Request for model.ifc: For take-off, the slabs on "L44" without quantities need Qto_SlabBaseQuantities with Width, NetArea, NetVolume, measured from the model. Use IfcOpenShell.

First a look at what the model holds.

```python
import ifcopenshell
import ifcopenshell.util.element
import ifcopenshell.util.unit

model = ifcopenshell.open("model.ifc")
print(model.schema)
for unit_type in ("LENGTHUNIT", "AREAUNIT", "VOLUMEUNIT"):
    print(unit_type, ifcopenshell.util.unit.calculate_unit_scale(model, unit_type))
storey = next(s for s in model.by_type("IfcBuildingStorey") if s.Name == "L44")
slabs = [e for e in ifcopenshell.util.element.get_decomposition(storey) if e.is_a("IfcSlab")]
for e in sorted(slabs, key=lambda e: e.id()):
    print(e.id(), e.is_a(), e.Name, list(ifcopenshell.util.element.get_psets(e, qtos_only=True)), sep=" | ")
```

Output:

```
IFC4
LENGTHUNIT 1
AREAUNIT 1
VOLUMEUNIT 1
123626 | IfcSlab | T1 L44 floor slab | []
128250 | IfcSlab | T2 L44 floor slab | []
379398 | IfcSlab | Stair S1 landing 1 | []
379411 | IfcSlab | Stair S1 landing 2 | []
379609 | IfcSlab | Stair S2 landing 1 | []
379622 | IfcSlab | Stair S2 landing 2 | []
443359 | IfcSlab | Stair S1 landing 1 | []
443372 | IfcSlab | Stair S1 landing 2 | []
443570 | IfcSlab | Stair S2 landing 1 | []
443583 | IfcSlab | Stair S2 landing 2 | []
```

```python
import ifcopenshell
import ifcopenshell.api.pset
import ifcopenshell.geom
import ifcopenshell.util.element
import ifcopenshell.util.shape
import ifcopenshell.util.unit

model = ifcopenshell.open("model.ifc")
unit_scale = ifcopenshell.util.unit.calculate_unit_scale(model)
area_scale = ifcopenshell.util.unit.calculate_unit_scale(model, "AREAUNIT")
volume_scale = ifcopenshell.util.unit.calculate_unit_scale(model, "VOLUMEUNIT")
settings = ifcopenshell.geom.settings()

storey = next(s for s in model.by_type("IfcBuildingStorey") if s.Name == "L44")
slabs = [e for e in ifcopenshell.util.element.get_decomposition(storey) if e.is_a("IfcSlab")]

for e in sorted(slabs, key=lambda e: e.id()):
    if ifcopenshell.util.element.get_psets(e, qtos_only=True, should_inherit=False):
        continue
    # Geometry comes back in metres, in the element's own axes.
    shape = ifcopenshell.geom.create_shape(settings, e)
    values = {
        "Width": ifcopenshell.util.shape.get_z(shape.geometry) / unit_scale,
        "NetArea": ifcopenshell.util.shape.get_footprint_area(shape.geometry) / area_scale,
        "NetVolume": ifcopenshell.util.shape.get_volume(shape.geometry) / volume_scale,
    }
    qto = ifcopenshell.api.pset.add_qto(model, product=e, name="Qto_SlabBaseQuantities")
    ifcopenshell.api.pset.edit_qto(model, qto=qto, properties=values)
    print(e.id(), {k: round(v, 3) for k, v in values.items()})

model.write("model-out.ifc")
```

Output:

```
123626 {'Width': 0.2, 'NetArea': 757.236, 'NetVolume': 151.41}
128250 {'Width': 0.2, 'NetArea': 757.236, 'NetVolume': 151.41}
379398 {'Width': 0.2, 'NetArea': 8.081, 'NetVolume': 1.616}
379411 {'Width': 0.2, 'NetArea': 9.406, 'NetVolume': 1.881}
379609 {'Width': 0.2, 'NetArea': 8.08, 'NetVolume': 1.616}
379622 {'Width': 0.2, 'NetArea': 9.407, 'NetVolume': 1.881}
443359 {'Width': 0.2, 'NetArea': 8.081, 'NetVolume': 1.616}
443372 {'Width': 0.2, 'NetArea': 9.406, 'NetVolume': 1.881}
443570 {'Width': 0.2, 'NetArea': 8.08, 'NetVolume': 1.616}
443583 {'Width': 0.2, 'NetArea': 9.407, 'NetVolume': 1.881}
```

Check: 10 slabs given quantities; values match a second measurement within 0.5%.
